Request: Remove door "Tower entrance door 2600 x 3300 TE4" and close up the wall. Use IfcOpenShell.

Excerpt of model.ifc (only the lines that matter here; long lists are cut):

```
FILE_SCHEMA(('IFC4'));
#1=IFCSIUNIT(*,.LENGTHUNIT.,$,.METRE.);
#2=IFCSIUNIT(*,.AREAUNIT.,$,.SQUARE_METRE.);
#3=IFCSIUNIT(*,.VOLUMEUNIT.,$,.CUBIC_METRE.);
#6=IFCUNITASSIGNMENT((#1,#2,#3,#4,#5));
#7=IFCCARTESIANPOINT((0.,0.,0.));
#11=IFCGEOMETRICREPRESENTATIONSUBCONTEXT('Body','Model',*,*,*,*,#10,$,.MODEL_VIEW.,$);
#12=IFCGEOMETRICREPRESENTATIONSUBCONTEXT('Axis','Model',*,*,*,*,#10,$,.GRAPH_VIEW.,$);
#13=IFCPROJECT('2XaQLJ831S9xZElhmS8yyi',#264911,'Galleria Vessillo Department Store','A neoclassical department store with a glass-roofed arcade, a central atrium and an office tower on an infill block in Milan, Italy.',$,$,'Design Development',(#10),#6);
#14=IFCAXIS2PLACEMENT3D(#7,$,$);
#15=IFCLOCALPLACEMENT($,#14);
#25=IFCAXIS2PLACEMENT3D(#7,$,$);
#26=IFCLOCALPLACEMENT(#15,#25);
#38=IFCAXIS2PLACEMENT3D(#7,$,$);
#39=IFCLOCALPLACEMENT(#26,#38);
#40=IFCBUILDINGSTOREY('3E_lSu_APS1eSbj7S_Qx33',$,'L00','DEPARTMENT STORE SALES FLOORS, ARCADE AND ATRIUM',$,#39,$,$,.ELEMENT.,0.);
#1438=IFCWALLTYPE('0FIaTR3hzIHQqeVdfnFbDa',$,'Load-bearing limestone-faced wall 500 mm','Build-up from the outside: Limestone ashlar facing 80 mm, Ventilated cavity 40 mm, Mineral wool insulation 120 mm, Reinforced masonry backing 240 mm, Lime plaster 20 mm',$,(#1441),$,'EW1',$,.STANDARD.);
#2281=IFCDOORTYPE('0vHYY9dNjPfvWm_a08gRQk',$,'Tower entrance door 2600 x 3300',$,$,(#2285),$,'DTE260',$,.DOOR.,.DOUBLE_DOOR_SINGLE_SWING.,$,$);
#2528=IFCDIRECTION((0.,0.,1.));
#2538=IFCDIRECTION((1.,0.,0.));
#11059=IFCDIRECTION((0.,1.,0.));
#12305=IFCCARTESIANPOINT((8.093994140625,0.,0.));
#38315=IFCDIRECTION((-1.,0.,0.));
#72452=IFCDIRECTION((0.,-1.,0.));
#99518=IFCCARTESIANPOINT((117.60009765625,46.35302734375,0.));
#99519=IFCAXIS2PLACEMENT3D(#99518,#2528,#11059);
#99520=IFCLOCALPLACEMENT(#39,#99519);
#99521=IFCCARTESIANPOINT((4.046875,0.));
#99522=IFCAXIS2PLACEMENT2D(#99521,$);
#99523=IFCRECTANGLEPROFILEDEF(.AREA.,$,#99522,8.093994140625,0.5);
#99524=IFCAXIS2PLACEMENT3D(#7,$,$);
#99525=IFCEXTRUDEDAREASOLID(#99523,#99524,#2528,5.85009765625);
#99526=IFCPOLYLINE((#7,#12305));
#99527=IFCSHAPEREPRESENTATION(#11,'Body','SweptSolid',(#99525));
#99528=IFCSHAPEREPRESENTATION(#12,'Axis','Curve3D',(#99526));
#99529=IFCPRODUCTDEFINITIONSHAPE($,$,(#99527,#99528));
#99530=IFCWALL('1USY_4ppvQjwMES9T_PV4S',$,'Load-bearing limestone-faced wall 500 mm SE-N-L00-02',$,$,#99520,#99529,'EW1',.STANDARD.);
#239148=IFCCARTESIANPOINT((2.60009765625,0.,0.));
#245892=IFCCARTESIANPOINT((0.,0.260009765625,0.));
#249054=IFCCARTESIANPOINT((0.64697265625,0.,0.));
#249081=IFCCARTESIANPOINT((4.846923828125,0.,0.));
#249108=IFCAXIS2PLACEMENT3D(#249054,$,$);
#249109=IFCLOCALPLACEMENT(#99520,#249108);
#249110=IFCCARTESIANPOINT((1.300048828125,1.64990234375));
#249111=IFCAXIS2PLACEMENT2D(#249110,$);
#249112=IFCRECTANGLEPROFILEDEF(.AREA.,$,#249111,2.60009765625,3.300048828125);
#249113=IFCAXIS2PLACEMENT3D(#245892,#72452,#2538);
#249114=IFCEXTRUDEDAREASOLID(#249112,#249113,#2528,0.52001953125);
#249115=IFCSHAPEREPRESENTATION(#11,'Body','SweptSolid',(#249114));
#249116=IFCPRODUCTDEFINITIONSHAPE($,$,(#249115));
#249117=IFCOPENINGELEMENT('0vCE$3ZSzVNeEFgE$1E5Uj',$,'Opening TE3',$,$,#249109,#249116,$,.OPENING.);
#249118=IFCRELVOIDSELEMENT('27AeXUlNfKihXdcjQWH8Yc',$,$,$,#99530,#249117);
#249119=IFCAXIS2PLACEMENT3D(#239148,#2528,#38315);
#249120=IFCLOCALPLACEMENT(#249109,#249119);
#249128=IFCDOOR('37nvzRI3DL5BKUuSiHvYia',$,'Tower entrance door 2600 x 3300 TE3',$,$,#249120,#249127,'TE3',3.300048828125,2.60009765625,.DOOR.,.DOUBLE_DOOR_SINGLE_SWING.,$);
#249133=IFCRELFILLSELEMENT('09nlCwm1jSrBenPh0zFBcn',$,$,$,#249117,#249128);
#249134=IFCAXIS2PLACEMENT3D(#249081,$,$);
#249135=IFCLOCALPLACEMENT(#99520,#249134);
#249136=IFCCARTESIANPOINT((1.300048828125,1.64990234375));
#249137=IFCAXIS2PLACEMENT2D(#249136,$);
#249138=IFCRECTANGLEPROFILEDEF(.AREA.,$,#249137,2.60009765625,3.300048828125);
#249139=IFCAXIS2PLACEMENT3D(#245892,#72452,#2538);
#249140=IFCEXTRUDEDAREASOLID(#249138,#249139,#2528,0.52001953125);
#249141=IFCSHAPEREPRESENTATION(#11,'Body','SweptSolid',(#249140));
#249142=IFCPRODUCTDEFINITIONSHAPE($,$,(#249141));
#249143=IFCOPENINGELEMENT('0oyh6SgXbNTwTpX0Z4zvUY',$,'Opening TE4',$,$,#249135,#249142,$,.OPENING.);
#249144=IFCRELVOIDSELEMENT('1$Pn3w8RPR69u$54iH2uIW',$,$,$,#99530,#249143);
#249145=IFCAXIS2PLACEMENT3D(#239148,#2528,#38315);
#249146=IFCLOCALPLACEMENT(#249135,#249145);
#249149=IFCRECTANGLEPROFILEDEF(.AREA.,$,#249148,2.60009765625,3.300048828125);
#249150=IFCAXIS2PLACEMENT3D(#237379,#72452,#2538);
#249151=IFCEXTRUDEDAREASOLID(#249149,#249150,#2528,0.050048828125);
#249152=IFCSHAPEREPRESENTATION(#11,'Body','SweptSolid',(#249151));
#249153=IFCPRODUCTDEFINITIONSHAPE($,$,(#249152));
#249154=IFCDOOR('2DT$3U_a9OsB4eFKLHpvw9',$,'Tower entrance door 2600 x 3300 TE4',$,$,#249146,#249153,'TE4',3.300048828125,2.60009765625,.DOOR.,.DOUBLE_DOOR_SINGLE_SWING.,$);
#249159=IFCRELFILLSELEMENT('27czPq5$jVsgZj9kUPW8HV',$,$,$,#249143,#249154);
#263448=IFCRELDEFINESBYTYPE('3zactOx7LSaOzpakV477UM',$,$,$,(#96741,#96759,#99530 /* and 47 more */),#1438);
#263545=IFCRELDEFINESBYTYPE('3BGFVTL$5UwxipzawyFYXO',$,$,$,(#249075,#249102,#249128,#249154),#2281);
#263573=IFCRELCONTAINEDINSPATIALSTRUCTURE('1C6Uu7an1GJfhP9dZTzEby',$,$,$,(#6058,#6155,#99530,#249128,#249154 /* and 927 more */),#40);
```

```python
import ifcopenshell
import ifcopenshell.api.feature
import ifcopenshell.api.root
import ifcopenshell.geom
import ifcopenshell.util.shape

model = ifcopenshell.open("model.ifc")
settings = ifcopenshell.geom.settings()


def volume(element):
    """Net volume in cubic metres, openings subtracted."""
    shape = ifcopenshell.geom.create_shape(settings, element)
    return ifcopenshell.util.shape.get_volume(shape.geometry)


door = model.by_guid("2DT$3U_a9OsB4eFKLHpvw9")
opening = door.FillsVoids[0].RelatingOpeningElement
wall = opening.VoidsElements[0].RelatingBuildingElement
before = volume(wall)

ifcopenshell.api.root.remove_product(model, product=door)
ifcopenshell.api.feature.remove_feature(model, feature=opening)

after = volume(wall)

print(f"wall volume {before:.3f} -> {after:.3f} m3")

model.write("model_rev.ifc")
```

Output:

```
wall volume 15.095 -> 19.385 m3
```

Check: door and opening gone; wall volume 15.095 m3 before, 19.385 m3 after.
